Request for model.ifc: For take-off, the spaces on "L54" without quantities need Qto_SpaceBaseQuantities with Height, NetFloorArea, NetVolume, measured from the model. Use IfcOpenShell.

First a look at what the model holds.

```python
import ifcopenshell
import ifcopenshell.util.element
import ifcopenshell.util.unit

model = ifcopenshell.open("model.ifc")
print(model.schema)
for unit_type in ("LENGTHUNIT", "AREAUNIT", "VOLUMEUNIT"):
    print(unit_type, ifcopenshell.util.unit.calculate_unit_scale(model, unit_type))
storey = next(s for s in model.by_type("IfcBuildingStorey") if s.Name == "L54")
spaces = [e for e in ifcopenshell.util.element.get_decomposition(storey) if e.is_a("IfcSpace")]
for e in sorted(spaces, key=lambda e: e.id()):
    print(e.id(), e.is_a(), e.Name, list(ifcopenshell.util.element.get_psets(e, qtos_only=True)), sep=" | ")
```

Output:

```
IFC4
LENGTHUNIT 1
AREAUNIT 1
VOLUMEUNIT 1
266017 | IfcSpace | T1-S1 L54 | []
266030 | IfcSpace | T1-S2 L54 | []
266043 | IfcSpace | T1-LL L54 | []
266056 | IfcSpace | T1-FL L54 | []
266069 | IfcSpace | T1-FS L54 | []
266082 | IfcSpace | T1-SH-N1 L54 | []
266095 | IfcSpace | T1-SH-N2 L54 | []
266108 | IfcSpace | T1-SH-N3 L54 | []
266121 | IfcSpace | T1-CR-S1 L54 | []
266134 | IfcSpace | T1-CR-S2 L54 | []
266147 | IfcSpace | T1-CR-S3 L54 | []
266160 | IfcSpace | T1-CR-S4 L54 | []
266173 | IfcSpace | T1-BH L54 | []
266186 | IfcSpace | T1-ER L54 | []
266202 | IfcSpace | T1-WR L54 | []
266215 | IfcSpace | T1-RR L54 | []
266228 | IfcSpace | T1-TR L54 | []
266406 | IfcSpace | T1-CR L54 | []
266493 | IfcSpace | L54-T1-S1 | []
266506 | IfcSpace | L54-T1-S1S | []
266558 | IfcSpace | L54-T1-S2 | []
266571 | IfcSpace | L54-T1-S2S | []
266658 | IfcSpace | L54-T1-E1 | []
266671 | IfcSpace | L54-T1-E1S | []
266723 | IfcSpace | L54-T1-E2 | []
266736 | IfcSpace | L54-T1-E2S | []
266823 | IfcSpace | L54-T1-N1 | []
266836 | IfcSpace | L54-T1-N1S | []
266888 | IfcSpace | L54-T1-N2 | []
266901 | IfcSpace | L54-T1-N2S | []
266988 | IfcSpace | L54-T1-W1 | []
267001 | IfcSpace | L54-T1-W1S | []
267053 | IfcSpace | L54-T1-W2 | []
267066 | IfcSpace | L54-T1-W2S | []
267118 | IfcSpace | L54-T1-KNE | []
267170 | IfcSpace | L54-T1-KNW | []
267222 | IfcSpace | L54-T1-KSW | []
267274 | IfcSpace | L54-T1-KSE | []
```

```python
import ifcopenshell
import ifcopenshell.api.pset
import ifcopenshell.geom
import ifcopenshell.util.element
import ifcopenshell.util.shape
import ifcopenshell.util.unit

model = ifcopenshell.open("model.ifc")
unit_scale = ifcopenshell.util.unit.calculate_unit_scale(model)
area_scale = ifcopenshell.util.unit.calculate_unit_scale(model, "AREAUNIT")
volume_scale = ifcopenshell.util.unit.calculate_unit_scale(model, "VOLUMEUNIT")
settings = ifcopenshell.geom.settings()

storey = next(s for s in model.by_type("IfcBuildingStorey") if s.Name == "L54")
spaces = [e for e in ifcopenshell.util.element.get_decomposition(storey) if e.is_a("IfcSpace")]

for e in sorted(spaces, key=lambda e: e.id()):
    if ifcopenshell.util.element.get_psets(e, qtos_only=True, should_inherit=False):
        continue
    # Geometry comes back in metres, in the element's own axes.
    shape = ifcopenshell.geom.create_shape(settings, e)
    values = {
        "Height": ifcopenshell.util.shape.get_z(shape.geometry) / unit_scale,
        "NetFloorArea": ifcopenshell.util.shape.get_footprint_area(shape.geometry) / area_scale,
        "NetVolume": ifcopenshell.util.shape.get_volume(shape.geometry) / volume_scale,
    }
    qto = ifcopenshell.api.pset.add_qto(model, product=e, name="Qto_SpaceBaseQuantities")
    ifcopenshell.api.pset.edit_qto(model, qto=qto, properties=values)
    print(e.id(), {k: round(v, 3) for k, v in values.items()})

model.write("model_updated.ifc")
```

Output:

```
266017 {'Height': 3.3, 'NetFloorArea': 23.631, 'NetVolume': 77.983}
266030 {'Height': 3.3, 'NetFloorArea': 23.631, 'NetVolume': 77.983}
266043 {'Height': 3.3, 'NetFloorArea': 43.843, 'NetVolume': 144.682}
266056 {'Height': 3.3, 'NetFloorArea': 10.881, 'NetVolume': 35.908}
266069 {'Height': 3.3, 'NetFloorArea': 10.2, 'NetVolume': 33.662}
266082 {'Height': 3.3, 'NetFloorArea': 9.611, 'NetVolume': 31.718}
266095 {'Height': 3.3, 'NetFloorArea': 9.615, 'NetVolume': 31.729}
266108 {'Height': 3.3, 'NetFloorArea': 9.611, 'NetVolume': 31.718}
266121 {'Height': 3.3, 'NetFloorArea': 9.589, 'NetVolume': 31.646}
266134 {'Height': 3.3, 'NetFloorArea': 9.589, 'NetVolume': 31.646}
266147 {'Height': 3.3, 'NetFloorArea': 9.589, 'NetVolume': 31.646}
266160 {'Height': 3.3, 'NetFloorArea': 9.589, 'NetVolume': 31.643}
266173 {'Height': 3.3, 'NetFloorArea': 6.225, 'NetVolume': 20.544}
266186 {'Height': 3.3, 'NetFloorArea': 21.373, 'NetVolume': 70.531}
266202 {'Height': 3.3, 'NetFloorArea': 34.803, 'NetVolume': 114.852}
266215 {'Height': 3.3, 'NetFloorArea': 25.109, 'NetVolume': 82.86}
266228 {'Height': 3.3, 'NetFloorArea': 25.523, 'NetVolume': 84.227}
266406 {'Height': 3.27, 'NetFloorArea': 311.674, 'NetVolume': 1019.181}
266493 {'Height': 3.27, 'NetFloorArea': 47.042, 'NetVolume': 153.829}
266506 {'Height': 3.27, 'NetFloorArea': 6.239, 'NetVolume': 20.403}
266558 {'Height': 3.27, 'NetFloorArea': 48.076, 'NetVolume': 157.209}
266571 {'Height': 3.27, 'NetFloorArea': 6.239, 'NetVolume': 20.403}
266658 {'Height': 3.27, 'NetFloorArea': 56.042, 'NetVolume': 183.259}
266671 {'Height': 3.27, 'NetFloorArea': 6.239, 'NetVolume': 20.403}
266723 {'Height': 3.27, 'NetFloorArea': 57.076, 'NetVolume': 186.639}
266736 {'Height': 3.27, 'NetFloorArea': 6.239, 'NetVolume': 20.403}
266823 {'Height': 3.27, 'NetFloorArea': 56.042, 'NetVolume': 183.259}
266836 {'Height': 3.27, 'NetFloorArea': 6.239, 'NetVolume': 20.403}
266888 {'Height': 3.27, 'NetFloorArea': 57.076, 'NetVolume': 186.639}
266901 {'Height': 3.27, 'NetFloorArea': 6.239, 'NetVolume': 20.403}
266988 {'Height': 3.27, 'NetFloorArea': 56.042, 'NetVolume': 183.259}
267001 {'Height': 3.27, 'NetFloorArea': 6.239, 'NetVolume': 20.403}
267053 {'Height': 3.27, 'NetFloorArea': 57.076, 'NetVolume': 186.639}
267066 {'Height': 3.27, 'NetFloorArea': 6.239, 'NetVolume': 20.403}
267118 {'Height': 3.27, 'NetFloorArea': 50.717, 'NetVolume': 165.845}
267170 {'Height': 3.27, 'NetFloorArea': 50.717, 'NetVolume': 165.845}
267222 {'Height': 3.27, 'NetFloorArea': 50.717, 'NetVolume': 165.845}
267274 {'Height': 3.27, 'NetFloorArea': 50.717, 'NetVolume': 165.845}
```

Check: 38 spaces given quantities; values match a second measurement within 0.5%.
